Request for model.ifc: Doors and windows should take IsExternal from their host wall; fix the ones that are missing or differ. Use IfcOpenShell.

First a look at what the model holds.

```python
import ifcopenshell
import ifcopenshell.util.element

model = ifcopenshell.open("model.ifc")
print(model.schema)
seen = {}
for e in model.by_type("IfcDoor") + model.by_type("IfcWindow"):
    if not e.FillsVoids:
        continue
    host = e.FillsVoids[0].RelatingOpeningElement.VoidsElements[0].RelatingBuildingElement
    own = ifcopenshell.util.element.get_pset(e, f"Pset_{e.is_a()[3:].removesuffix('StandardCase')}Common", "IsExternal")
    wall = ifcopenshell.util.element.get_pset(host, "Pset_WallCommon", "IsExternal")
    seen[e.is_a(), own, wall] = seen.get((e.is_a(), own, wall), 0) + 1
for (cls, own, wall), count in sorted(seen.items(), key=str):
    print(count, cls, "IsExternal:", own, "| host wall:", wall)
```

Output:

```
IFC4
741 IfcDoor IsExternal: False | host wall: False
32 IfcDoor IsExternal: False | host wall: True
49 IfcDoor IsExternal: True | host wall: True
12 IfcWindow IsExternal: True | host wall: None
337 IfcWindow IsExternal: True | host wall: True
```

```python
import ifcopenshell
import ifcopenshell.api.pset
import ifcopenshell.util.element

model = ifcopenshell.open("model.ifc")

count = 0
for ifc_class, pset_name in (("IfcDoor", "Pset_DoorCommon"), ("IfcWindow", "Pset_WindowCommon")):
    for e in model.by_type(ifc_class):
        if not e.FillsVoids:
            continue
        host = e.FillsVoids[0].RelatingOpeningElement.VoidsElements[0].RelatingBuildingElement
        external = ifcopenshell.util.element.get_pset(host, "Pset_WallCommon", "IsExternal")
        if external is None or ifcopenshell.util.element.get_pset(e, pset_name, "IsExternal") == external:
            continue
        pset = ifcopenshell.api.pset.add_pset(model, product=e, name=pset_name)
        ifcopenshell.api.pset.edit_pset(model, pset=pset, properties={"IsExternal": external})
        count += 1

print(count, "updated")

model.write("model_updated.ifc")
```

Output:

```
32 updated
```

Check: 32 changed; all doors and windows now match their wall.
